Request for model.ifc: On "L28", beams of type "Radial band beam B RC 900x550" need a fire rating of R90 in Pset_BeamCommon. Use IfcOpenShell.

First a look at what the model holds.

```python
import ifcopenshell
import ifcopenshell.util.element

model = ifcopenshell.open("model.ifc")
print(model.schema)
storey = next(s for s in model.by_type("IfcBuildingStorey") if s.Name == "L28")
beams = [e for e in ifcopenshell.util.element.get_decomposition(storey) if e.is_a("IfcBeam")]
seen = {}
for e in beams:
    element_type = ifcopenshell.util.element.get_type(e)
    key = (element_type.Name if element_type != e and element_type else None, ifcopenshell.util.element.get_pset(e, "Pset_BeamCommon", "FireRating"))
    seen[key] = seen.get(key, 0) + 1
for (name, value), count in sorted(seen.items(), key=str):
    print(count, "x", name, "|", value)
```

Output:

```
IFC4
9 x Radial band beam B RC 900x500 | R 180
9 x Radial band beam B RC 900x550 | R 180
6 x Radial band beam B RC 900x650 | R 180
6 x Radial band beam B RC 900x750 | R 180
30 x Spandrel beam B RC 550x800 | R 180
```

```python
import ifcopenshell
import ifcopenshell.api.pset
import ifcopenshell.util.element

model = ifcopenshell.open("model.ifc")

storey = next(s for s in model.by_type("IfcBuildingStorey") if s.Name == "L28")
beams = [e for e in ifcopenshell.util.element.get_decomposition(storey) if e.is_a("IfcBeam")]

count = 0
for e in beams:
    element_type = ifcopenshell.util.element.get_type(e)
    if element_type in (None, e) or element_type.Name != "Radial band beam B RC 900x550":
        continue
    found = ifcopenshell.util.element.get_pset(e, "Pset_BeamCommon", should_inherit=False)
    if found:
        pset = model.by_id(found["id"])
        if len(ifcopenshell.util.element.get_elements_by_pset(pset)) > 1:
            pset = ifcopenshell.api.pset.unshare_pset(model, products=[e], pset=pset)[0]
    else:
        pset = ifcopenshell.api.pset.add_pset(model, product=e, name="Pset_BeamCommon")
    ifcopenshell.api.pset.edit_pset(model, pset=pset, properties={"FireRating": "R90"})
    count += 1

print(count, "beams updated")

model.write("model-out.ifc")
```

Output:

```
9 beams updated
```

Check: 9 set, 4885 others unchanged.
